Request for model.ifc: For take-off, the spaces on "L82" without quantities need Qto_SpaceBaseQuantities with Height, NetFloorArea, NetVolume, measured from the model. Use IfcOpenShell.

First a look at what the model holds.

```python
import ifcopenshell
import ifcopenshell.util.element
import ifcopenshell.util.unit

model = ifcopenshell.open("model.ifc")
print(model.schema)
for unit_type in ("LENGTHUNIT", "AREAUNIT", "VOLUMEUNIT"):
    print(unit_type, ifcopenshell.util.unit.calculate_unit_scale(model, unit_type))
storey = next(s for s in model.by_type("IfcBuildingStorey") if s.Name == "L82")
spaces = [e for e in ifcopenshell.util.element.get_decomposition(storey) if e.is_a("IfcSpace")]
for e in sorted(spaces, key=lambda e: e.id()):
    print(e.id(), e.is_a(), e.Name, list(ifcopenshell.util.element.get_psets(e, qtos_only=True)), sep=" | ")
```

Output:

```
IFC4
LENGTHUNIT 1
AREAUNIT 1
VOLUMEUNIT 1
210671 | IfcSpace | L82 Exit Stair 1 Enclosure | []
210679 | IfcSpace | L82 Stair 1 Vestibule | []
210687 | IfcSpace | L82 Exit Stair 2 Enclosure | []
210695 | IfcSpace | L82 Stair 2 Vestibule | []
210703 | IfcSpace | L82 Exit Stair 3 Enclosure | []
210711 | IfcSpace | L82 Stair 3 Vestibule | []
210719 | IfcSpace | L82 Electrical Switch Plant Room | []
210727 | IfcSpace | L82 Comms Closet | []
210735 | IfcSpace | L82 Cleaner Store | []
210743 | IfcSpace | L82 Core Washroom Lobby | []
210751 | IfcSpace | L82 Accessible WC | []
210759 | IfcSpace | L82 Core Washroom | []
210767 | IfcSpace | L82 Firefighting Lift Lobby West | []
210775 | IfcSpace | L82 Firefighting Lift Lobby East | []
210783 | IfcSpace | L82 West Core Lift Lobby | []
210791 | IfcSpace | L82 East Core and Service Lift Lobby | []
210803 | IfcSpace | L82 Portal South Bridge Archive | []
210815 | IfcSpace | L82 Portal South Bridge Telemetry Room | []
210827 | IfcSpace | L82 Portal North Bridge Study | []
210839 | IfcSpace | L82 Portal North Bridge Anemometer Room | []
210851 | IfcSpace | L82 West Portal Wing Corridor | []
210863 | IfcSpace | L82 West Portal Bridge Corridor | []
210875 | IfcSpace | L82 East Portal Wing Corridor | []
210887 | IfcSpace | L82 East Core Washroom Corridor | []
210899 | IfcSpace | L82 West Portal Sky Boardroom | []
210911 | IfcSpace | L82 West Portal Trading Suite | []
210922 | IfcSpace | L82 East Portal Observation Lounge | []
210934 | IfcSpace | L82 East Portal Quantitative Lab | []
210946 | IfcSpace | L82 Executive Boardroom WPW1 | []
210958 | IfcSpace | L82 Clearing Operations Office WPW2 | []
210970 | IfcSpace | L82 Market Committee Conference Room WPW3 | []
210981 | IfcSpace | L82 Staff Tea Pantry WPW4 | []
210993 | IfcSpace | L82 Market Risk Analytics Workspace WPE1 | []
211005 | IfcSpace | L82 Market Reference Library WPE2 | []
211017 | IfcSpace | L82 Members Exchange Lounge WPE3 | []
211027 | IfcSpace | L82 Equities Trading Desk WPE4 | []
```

```python
import ifcopenshell
import ifcopenshell.api.pset
import ifcopenshell.geom
import ifcopenshell.util.element
import ifcopenshell.util.shape
import ifcopenshell.util.unit

model = ifcopenshell.open("model.ifc")
unit_scale = ifcopenshell.util.unit.calculate_unit_scale(model)
area_scale = ifcopenshell.util.unit.calculate_unit_scale(model, "AREAUNIT")
volume_scale = ifcopenshell.util.unit.calculate_unit_scale(model, "VOLUMEUNIT")
settings = ifcopenshell.geom.settings()

storey = next(s for s in model.by_type("IfcBuildingStorey") if s.Name == "L82")
spaces = [e for e in ifcopenshell.util.element.get_decomposition(storey) if e.is_a("IfcSpace")]

for e in sorted(spaces, key=lambda e: e.id()):
    if ifcopenshell.util.element.get_psets(e, qtos_only=True, should_inherit=False):
        continue
    # Geometry comes back in metres, in the element's own axes.
    shape = ifcopenshell.geom.create_shape(settings, e)
    values = {
        "Height": ifcopenshell.util.shape.get_z(shape.geometry) / unit_scale,
        "NetFloorArea": ifcopenshell.util.shape.get_footprint_area(shape.geometry) / area_scale,
        "NetVolume": ifcopenshell.util.shape.get_volume(shape.geometry) / volume_scale,
    }
    qto = ifcopenshell.api.pset.add_qto(model, product=e, name="Qto_SpaceBaseQuantities")
    ifcopenshell.api.pset.edit_qto(model, qto=qto, properties=values)
    print(e.id(), {k: round(v, 3) for k, v in values.items()})

model.write("model_rev.ifc")
```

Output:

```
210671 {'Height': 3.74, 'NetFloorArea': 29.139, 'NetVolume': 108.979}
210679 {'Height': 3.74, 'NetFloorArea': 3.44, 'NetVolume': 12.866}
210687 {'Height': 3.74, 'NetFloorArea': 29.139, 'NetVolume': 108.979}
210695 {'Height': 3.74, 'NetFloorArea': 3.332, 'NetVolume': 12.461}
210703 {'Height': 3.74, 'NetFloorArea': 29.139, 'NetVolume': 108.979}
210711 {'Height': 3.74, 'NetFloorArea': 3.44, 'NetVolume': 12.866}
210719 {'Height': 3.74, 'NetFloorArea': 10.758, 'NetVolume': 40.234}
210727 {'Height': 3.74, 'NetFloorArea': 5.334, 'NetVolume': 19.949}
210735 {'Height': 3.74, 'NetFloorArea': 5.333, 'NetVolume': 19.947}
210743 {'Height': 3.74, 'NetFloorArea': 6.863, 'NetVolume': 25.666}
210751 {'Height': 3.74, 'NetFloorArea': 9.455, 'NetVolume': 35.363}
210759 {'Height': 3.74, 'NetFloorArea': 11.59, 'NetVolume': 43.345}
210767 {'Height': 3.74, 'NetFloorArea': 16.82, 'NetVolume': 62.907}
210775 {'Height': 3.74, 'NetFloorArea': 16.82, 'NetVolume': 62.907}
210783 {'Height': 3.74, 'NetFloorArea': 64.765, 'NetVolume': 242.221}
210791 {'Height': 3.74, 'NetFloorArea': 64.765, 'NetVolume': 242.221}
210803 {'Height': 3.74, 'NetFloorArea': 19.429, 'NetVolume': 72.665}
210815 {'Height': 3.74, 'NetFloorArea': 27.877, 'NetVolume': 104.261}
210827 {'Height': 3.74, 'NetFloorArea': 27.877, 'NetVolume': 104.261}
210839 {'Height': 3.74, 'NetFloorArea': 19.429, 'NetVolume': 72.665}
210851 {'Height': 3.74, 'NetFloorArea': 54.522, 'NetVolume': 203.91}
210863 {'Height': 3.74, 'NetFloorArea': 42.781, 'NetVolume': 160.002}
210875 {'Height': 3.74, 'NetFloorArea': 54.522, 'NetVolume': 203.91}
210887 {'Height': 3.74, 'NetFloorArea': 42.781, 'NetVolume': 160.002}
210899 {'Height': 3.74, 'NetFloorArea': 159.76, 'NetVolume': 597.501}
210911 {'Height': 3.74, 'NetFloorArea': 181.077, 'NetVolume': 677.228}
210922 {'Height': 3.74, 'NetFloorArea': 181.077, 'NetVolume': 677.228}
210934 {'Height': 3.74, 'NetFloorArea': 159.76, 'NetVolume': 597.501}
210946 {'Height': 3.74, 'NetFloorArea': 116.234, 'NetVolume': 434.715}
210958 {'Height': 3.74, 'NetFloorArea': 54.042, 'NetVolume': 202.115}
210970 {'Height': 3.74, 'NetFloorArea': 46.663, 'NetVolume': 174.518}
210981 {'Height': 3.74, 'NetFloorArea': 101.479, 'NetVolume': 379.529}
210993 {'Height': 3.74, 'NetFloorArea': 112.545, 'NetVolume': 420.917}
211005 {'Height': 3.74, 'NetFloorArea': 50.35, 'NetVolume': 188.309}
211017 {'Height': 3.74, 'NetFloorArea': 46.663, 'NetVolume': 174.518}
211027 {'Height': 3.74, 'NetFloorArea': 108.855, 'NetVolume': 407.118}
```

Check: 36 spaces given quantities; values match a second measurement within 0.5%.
